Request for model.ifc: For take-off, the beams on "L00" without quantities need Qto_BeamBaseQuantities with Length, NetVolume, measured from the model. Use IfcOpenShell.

First a look at what the model holds.

```python
import ifcopenshell
import ifcopenshell.util.element
import ifcopenshell.util.unit

model = ifcopenshell.open("model.ifc")
print(model.schema)
for unit_type in ("LENGTHUNIT", "AREAUNIT", "VOLUMEUNIT"):
    print(unit_type, ifcopenshell.util.unit.calculate_unit_scale(model, unit_type))
storey = next(s for s in model.by_type("IfcBuildingStorey") if s.Name == "L00")
beams = [e for e in ifcopenshell.util.element.get_decomposition(storey) if e.is_a("IfcBeam")]
for e in sorted(beams, key=lambda e: e.id()):
    print(e.id(), e.is_a(), e.Name, list(ifcopenshell.util.element.get_psets(e, qtos_only=True)), sep=" | ")
```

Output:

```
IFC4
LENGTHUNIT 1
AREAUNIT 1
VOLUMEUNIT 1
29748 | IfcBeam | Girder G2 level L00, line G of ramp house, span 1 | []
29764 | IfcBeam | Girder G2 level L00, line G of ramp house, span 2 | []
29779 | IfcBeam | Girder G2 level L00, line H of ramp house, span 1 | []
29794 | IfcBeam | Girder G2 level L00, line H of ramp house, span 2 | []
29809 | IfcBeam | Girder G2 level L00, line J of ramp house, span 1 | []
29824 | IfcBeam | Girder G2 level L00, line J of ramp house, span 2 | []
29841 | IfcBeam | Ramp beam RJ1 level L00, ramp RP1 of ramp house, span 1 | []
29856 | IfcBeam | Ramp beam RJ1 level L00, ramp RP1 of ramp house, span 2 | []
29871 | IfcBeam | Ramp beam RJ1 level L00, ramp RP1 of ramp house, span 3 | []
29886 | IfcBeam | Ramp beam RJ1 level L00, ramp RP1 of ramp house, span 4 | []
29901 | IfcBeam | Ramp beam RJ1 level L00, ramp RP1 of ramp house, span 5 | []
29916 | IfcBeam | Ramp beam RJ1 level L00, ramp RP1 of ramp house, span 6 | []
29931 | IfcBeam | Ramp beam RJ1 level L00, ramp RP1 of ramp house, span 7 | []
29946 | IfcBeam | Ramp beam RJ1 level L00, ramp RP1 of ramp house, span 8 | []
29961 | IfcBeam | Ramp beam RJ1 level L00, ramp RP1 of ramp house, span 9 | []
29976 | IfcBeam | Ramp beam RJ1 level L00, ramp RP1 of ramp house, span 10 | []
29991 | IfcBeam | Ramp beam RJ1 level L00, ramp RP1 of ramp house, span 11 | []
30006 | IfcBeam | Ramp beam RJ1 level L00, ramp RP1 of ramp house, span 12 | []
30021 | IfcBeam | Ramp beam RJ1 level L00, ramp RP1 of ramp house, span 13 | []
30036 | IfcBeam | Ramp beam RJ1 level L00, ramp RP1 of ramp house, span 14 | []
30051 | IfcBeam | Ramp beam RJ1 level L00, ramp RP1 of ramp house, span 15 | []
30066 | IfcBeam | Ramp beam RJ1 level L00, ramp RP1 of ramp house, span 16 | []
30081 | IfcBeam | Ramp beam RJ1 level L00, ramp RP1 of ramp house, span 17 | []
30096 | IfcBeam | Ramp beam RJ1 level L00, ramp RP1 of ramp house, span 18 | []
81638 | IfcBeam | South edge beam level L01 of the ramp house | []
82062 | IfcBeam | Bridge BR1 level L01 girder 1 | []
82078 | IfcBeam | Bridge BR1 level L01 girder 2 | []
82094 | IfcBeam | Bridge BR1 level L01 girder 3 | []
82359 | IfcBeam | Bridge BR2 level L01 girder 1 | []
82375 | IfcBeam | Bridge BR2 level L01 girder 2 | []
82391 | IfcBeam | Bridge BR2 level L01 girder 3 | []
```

```python
import ifcopenshell
import ifcopenshell.api.pset
import ifcopenshell.geom
import ifcopenshell.util.element
import ifcopenshell.util.shape
import ifcopenshell.util.unit

model = ifcopenshell.open("model.ifc")
unit_scale = ifcopenshell.util.unit.calculate_unit_scale(model)
volume_scale = ifcopenshell.util.unit.calculate_unit_scale(model, "VOLUMEUNIT")
settings = ifcopenshell.geom.settings()

storey = next(s for s in model.by_type("IfcBuildingStorey") if s.Name == "L00")
beams = [e for e in ifcopenshell.util.element.get_decomposition(storey) if e.is_a("IfcBeam")]

for e in sorted(beams, key=lambda e: e.id()):
    if ifcopenshell.util.element.get_psets(e, qtos_only=True, should_inherit=False):
        continue
    # Geometry comes back in metres, in the element's own axes.
    shape = ifcopenshell.geom.create_shape(settings, e)
    values = {
        "Length": ifcopenshell.util.shape.get_max_xyz(shape.geometry) / unit_scale,
        "NetVolume": ifcopenshell.util.shape.get_volume(shape.geometry) / volume_scale,
    }
    qto = ifcopenshell.api.pset.add_qto(model, product=e, name="Qto_BeamBaseQuantities")
    ifcopenshell.api.pset.edit_qto(model, qto=qto, properties=values)
    print(e.id(), {k: round(v, 3) for k, v in values.items()})

model.write("model_edited.ifc")
```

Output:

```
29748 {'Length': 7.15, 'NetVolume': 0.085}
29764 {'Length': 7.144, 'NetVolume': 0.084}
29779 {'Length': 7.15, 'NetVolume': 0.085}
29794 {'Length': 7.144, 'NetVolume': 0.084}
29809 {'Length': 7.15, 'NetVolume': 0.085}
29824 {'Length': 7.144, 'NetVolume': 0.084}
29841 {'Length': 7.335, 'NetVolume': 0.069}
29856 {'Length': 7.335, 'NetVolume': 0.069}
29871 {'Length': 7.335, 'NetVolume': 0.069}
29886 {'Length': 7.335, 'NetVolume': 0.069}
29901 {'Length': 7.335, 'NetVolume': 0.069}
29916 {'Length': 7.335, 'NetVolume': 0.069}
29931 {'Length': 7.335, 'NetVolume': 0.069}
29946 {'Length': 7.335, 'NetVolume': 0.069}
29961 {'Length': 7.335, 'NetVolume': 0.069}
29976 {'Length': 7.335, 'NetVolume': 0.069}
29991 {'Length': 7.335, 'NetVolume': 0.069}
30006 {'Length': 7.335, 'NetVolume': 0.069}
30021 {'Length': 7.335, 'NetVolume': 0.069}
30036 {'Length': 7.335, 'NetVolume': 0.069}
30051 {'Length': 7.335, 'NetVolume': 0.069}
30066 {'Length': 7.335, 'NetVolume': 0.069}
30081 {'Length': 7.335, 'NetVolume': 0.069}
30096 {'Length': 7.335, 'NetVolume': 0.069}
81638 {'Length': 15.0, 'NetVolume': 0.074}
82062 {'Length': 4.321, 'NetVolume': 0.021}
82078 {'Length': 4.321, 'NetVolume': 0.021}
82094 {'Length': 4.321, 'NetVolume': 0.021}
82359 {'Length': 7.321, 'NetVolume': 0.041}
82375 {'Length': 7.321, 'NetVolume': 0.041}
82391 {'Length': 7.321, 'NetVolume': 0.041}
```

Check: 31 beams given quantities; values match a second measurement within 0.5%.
